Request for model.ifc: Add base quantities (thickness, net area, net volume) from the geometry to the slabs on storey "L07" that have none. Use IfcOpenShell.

First a look at what the model holds.

```python
import ifcopenshell
import ifcopenshell.util.element
import ifcopenshell.util.unit

model = ifcopenshell.open("model.ifc")
print(model.schema)
for unit_type in ("LENGTHUNIT", "AREAUNIT", "VOLUMEUNIT"):
    print(unit_type, ifcopenshell.util.unit.calculate_unit_scale(model, unit_type))
storey = next(s for s in model.by_type("IfcBuildingStorey") if s.Name == "L07")
slabs = [e for e in ifcopenshell.util.element.get_decomposition(storey) if e.is_a("IfcSlab")]
for e in sorted(slabs, key=lambda e: e.id()):
    print(e.id(), e.is_a(), e.Name, list(ifcopenshell.util.element.get_psets(e, qtos_only=True)), sep=" | ")
```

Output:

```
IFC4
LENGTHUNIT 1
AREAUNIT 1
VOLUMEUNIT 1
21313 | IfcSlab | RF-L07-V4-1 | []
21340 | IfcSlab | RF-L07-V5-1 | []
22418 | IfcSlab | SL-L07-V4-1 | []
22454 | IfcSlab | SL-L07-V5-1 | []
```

```python
import ifcopenshell
import ifcopenshell.api.pset
import ifcopenshell.geom
import ifcopenshell.util.element
import ifcopenshell.util.shape
import ifcopenshell.util.unit

model = ifcopenshell.open("model.ifc")
unit_scale = ifcopenshell.util.unit.calculate_unit_scale(model)
area_scale = ifcopenshell.util.unit.calculate_unit_scale(model, "AREAUNIT")
volume_scale = ifcopenshell.util.unit.calculate_unit_scale(model, "VOLUMEUNIT")
settings = ifcopenshell.geom.settings()

storey = next(s for s in model.by_type("IfcBuildingStorey") if s.Name == "L07")
slabs = [e for e in ifcopenshell.util.element.get_decomposition(storey) if e.is_a("IfcSlab")]

for e in sorted(slabs, key=lambda e: e.id()):
    if ifcopenshell.util.element.get_psets(e, qtos_only=True, should_inherit=False):
        continue
    # Geometry comes back in metres, in the element's own axes.
    shape = ifcopenshell.geom.create_shape(settings, e)
    values = {
        "Width": ifcopenshell.util.shape.get_z(shape.geometry) / unit_scale,
        "NetArea": ifcopenshell.util.shape.get_footprint_area(shape.geometry) / area_scale,
        "NetVolume": ifcopenshell.util.shape.get_volume(shape.geometry) / volume_scale,
    }
    qto = ifcopenshell.api.pset.add_qto(model, product=e, name="Qto_SlabBaseQuantities")
    ifcopenshell.api.pset.edit_qto(model, qto=qto, properties=values)
    print(e.id(), {k: round(v, 3) for k, v in values.items()})

model.write("model-out.ifc")
```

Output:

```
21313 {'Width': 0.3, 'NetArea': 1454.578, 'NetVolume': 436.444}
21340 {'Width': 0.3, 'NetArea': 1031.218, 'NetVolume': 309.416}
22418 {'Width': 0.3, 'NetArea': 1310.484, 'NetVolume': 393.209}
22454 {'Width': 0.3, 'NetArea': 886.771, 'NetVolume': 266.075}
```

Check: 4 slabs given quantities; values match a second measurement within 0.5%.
